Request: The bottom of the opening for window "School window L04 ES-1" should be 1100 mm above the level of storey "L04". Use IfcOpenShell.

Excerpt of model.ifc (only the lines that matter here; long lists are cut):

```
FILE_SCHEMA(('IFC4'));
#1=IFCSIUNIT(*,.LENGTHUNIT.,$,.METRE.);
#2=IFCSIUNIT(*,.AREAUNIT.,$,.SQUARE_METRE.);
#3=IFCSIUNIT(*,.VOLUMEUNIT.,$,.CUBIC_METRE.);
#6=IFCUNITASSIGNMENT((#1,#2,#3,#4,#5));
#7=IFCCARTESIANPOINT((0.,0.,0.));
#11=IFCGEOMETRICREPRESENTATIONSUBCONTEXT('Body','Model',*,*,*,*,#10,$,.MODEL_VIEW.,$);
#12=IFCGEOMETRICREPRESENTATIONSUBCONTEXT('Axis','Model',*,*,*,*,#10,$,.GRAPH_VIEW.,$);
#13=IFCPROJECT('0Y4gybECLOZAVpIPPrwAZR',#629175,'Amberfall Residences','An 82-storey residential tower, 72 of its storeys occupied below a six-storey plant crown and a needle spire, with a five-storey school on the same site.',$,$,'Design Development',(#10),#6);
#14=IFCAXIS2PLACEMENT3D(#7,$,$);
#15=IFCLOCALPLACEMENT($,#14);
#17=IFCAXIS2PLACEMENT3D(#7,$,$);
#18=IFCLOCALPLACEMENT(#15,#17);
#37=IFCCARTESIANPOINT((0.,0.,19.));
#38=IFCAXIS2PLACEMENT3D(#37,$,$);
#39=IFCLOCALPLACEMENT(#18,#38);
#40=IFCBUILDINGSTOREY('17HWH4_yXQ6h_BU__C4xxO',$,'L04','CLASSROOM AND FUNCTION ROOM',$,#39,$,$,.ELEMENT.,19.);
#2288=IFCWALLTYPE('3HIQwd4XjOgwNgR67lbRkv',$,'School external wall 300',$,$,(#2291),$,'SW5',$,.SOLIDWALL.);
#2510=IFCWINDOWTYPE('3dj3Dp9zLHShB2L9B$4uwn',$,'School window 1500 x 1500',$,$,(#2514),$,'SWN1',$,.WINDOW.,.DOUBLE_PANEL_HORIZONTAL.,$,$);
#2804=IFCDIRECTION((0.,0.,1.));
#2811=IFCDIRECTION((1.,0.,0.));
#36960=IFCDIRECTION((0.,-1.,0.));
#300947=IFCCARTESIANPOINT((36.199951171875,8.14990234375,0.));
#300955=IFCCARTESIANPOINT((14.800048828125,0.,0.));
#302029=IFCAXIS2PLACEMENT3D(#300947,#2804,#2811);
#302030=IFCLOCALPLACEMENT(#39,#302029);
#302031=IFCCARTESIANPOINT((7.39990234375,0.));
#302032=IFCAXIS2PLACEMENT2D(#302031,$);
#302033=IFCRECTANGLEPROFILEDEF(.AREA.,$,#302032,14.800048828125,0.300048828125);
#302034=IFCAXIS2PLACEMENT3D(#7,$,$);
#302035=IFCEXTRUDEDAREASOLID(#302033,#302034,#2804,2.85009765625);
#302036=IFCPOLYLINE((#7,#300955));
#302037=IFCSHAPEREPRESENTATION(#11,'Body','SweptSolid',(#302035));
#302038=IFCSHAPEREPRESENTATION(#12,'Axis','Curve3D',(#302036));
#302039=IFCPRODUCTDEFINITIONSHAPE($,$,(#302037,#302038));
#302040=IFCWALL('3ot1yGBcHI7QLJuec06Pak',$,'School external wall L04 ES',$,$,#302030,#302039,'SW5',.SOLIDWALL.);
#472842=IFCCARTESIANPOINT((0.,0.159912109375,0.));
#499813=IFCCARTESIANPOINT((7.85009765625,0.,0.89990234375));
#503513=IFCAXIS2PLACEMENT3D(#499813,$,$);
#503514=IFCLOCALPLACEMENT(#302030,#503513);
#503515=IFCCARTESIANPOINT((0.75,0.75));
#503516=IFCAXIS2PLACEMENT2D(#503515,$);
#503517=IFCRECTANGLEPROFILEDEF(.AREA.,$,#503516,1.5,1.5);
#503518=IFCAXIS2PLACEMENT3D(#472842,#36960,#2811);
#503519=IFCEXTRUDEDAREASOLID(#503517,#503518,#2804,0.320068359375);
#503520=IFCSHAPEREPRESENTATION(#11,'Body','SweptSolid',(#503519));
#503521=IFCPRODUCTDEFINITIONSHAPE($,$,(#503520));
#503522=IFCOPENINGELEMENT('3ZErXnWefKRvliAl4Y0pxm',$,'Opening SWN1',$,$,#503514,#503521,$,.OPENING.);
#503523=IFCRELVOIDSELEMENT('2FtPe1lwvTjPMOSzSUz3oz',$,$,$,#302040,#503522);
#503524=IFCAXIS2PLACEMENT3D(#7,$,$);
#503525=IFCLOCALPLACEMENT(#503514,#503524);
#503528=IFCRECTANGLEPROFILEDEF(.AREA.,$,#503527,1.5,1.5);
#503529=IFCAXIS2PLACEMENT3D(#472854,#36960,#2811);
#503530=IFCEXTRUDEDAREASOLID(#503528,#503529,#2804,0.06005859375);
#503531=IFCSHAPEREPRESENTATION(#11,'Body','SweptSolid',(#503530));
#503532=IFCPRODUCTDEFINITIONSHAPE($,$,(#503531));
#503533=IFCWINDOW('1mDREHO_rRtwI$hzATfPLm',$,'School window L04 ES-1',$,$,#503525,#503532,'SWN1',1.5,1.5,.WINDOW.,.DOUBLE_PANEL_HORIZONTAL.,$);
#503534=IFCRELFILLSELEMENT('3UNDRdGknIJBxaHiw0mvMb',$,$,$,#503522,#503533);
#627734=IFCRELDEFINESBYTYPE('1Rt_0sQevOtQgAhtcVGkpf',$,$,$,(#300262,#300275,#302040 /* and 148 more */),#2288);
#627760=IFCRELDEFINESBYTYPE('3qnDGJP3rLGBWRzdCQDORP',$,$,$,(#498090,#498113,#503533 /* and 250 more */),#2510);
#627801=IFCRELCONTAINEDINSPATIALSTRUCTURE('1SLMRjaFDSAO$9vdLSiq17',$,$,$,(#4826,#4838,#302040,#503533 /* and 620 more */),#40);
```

```python
import numpy as np
import ifcopenshell
import ifcopenshell.api.geometry
import ifcopenshell.geom
import ifcopenshell.util.element
import ifcopenshell.util.placement
import ifcopenshell.util.shape
import ifcopenshell.util.unit

model = ifcopenshell.open("model.ifc")
unit_scale = ifcopenshell.util.unit.calculate_unit_scale(model)

window = model.by_guid("1mDREHO_rRtwI$hzATfPLm")
opening = window.FillsVoids[0].RelatingOpeningElement
storey = ifcopenshell.util.element.get_container(window, ifc_class="IfcBuildingStorey")
level = ifcopenshell.util.placement.get_local_placement(storey.ObjectPlacement)[2, 3]

# The opening's origin need not be at the sill, so measure its lowest point.
shape = ifcopenshell.geom.create_shape(ifcopenshell.geom.settings(), opening)
bottom = ifcopenshell.util.shape.get_shape_bottom_elevation(shape, shape.geometry) / unit_scale
dz = level + 1.1 - bottom

shift = np.array([0.0, 0.0, dz])
# The window is placed relative to its opening, so it follows when the opening moves.
matrix = ifcopenshell.util.placement.get_local_placement(opening.ObjectPlacement)
matrix[:3, 3] += shift
ifcopenshell.api.geometry.edit_object_placement(
    model, product=opening, matrix=matrix, is_si=False, should_transform_children=True
)

print(f"moved by {dz * unit_scale:+.3f} m")

model.write("model_edited.ifc")
```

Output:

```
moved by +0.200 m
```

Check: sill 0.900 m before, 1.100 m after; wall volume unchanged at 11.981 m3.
